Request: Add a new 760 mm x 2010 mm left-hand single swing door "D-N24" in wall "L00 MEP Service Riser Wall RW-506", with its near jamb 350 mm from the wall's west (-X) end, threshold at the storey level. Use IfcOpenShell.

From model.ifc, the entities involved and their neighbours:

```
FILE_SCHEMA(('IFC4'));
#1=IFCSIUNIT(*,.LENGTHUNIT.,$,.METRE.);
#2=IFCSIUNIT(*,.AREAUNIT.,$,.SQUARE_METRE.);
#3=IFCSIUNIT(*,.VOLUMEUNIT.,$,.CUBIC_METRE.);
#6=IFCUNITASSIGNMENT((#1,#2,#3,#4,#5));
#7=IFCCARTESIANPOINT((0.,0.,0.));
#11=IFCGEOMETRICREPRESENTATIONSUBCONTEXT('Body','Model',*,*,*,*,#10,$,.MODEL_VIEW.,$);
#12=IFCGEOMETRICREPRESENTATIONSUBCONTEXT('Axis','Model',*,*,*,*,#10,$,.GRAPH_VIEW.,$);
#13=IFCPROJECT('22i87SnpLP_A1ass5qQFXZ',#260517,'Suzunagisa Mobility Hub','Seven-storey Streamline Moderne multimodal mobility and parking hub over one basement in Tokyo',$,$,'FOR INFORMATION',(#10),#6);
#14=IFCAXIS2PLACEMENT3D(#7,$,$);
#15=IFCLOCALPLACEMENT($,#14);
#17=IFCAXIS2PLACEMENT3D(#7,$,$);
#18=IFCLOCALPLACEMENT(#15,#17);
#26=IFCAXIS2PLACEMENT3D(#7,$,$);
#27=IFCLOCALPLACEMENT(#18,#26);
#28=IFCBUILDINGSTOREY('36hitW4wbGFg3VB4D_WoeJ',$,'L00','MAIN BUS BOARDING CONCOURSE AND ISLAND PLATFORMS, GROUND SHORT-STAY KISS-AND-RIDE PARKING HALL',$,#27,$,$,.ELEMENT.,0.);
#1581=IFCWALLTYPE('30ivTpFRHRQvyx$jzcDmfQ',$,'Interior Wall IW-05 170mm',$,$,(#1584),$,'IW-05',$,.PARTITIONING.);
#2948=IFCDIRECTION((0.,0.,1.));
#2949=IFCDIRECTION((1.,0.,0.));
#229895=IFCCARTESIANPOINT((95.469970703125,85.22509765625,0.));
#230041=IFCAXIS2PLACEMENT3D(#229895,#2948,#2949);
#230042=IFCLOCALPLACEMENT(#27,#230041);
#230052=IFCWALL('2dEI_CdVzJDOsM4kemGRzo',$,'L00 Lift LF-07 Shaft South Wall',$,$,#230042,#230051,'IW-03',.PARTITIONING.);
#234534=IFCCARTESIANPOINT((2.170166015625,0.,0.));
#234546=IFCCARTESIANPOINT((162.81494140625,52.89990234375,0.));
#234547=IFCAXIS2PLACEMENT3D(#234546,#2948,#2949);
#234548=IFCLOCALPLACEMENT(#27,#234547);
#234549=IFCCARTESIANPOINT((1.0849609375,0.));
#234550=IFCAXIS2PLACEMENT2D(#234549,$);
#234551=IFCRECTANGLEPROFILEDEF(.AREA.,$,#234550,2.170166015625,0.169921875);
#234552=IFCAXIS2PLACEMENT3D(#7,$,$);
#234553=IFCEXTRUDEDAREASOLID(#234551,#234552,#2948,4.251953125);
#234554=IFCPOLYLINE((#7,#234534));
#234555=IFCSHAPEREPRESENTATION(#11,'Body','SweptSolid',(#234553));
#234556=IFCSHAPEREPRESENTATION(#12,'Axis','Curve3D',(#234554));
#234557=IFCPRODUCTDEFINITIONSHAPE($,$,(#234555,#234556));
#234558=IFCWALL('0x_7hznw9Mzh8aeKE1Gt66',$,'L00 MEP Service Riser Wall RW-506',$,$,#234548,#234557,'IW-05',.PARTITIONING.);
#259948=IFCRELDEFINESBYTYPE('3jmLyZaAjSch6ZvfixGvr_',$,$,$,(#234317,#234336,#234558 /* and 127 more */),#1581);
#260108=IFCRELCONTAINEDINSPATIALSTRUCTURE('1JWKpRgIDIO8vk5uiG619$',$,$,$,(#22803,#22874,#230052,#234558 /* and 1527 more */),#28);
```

```python
import numpy as np
import ifcopenshell
import ifcopenshell.api.feature
import ifcopenshell.api.geometry
import ifcopenshell.api.root
import ifcopenshell.api.spatial
import ifcopenshell.geom
import ifcopenshell.util.element
import ifcopenshell.util.placement
import ifcopenshell.util.representation
import ifcopenshell.util.shape
import ifcopenshell.util.unit

model = ifcopenshell.open("model.ifc")
unit_scale = ifcopenshell.util.unit.calculate_unit_scale(model)
settings = ifcopenshell.geom.settings()


def volume(element):
    """Net volume in cubic metres, openings subtracted."""
    shape = ifcopenshell.geom.create_shape(settings, element)
    return ifcopenshell.util.shape.get_volume(shape.geometry)


wall = model.by_guid("0x_7hznw9Mzh8aeKE1Gt66")
storey = ifcopenshell.util.element.get_container(wall, ifc_class="IfcBuildingStorey")
context = ifcopenshell.util.representation.get_context(model, "Model", "Body", "MODEL_VIEW")
before = volume(wall)

width, height, from_end, sill = 0.76, 2.01, 0.35, 0.0  # metres

# The wall runs along its own X axis, and the end named is its -X end.
wall_shape = ifcopenshell.geom.create_shape(settings, wall)
x, y, z = ifcopenshell.util.shape.get_vertices(wall_shape.geometry).T
start = x.min() + from_end
face, thickness = float(y.min()), float(y.max() - y.min())
wall_matrix = ifcopenshell.util.placement.get_local_placement(wall.ObjectPlacement)
level = ifcopenshell.util.placement.get_local_placement(storey.ObjectPlacement)[2, 3]


def in_wall(x, y):
    """Placement at x, y metres in the wall's axes, at sill height."""
    matrix = wall_matrix.copy()
    matrix[:, 3] = wall_matrix @ np.array([x / unit_scale, y / unit_scale, 0.0, 1.0])
    matrix[2, 3] = level + sill / unit_scale
    return matrix


# Opening: a box that overshoots both wall faces by 50 mm.
opening = ifcopenshell.api.root.create_entity(model, ifc_class="IfcOpeningElement", predefined_type="OPENING")
box = ifcopenshell.api.geometry.add_wall_representation(
    model, context=context, length=width, height=height, thickness=thickness + 0.1
)
ifcopenshell.api.geometry.assign_representation(model, product=opening, representation=box)
ifcopenshell.api.geometry.edit_object_placement(model, product=opening, matrix=in_wall(start, face - 0.05), is_si=False)
ifcopenshell.api.feature.add_feature(model, feature=opening, element=wall)

door = ifcopenshell.api.root.create_entity(model, ifc_class="IfcDoor", name="D-N24", predefined_type="DOOR")
door.OverallWidth, door.OverallHeight = width / unit_scale, height / unit_scale
door.OperationType = "SINGLE_SWING_LEFT"
body = ifcopenshell.api.geometry.add_door_representation(
    model,
    context=context,
    overall_width=door.OverallWidth,
    overall_height=door.OverallHeight,
    operation_type="SINGLE_SWING_LEFT",
    lining_properties={"LiningDepth": thickness / unit_scale, "ThresholdDepth": thickness / unit_scale},
)
ifcopenshell.api.geometry.assign_representation(model, product=door, representation=body)
ifcopenshell.api.spatial.assign_container(model, products=[door], relating_structure=storey)
ifcopenshell.api.feature.add_filling(model, opening=opening, element=door)

# The lining spans the wall, so the door starts at the wall face.
ifcopenshell.api.geometry.edit_object_placement(model, product=door, matrix=in_wall(start, face), is_si=False)

after = volume(wall)

print(f"wall volume {before:.3f} -> {after:.3f} m3")

model.write("model_edited.ifc")
```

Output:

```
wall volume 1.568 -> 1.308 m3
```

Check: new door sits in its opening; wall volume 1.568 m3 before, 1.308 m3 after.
